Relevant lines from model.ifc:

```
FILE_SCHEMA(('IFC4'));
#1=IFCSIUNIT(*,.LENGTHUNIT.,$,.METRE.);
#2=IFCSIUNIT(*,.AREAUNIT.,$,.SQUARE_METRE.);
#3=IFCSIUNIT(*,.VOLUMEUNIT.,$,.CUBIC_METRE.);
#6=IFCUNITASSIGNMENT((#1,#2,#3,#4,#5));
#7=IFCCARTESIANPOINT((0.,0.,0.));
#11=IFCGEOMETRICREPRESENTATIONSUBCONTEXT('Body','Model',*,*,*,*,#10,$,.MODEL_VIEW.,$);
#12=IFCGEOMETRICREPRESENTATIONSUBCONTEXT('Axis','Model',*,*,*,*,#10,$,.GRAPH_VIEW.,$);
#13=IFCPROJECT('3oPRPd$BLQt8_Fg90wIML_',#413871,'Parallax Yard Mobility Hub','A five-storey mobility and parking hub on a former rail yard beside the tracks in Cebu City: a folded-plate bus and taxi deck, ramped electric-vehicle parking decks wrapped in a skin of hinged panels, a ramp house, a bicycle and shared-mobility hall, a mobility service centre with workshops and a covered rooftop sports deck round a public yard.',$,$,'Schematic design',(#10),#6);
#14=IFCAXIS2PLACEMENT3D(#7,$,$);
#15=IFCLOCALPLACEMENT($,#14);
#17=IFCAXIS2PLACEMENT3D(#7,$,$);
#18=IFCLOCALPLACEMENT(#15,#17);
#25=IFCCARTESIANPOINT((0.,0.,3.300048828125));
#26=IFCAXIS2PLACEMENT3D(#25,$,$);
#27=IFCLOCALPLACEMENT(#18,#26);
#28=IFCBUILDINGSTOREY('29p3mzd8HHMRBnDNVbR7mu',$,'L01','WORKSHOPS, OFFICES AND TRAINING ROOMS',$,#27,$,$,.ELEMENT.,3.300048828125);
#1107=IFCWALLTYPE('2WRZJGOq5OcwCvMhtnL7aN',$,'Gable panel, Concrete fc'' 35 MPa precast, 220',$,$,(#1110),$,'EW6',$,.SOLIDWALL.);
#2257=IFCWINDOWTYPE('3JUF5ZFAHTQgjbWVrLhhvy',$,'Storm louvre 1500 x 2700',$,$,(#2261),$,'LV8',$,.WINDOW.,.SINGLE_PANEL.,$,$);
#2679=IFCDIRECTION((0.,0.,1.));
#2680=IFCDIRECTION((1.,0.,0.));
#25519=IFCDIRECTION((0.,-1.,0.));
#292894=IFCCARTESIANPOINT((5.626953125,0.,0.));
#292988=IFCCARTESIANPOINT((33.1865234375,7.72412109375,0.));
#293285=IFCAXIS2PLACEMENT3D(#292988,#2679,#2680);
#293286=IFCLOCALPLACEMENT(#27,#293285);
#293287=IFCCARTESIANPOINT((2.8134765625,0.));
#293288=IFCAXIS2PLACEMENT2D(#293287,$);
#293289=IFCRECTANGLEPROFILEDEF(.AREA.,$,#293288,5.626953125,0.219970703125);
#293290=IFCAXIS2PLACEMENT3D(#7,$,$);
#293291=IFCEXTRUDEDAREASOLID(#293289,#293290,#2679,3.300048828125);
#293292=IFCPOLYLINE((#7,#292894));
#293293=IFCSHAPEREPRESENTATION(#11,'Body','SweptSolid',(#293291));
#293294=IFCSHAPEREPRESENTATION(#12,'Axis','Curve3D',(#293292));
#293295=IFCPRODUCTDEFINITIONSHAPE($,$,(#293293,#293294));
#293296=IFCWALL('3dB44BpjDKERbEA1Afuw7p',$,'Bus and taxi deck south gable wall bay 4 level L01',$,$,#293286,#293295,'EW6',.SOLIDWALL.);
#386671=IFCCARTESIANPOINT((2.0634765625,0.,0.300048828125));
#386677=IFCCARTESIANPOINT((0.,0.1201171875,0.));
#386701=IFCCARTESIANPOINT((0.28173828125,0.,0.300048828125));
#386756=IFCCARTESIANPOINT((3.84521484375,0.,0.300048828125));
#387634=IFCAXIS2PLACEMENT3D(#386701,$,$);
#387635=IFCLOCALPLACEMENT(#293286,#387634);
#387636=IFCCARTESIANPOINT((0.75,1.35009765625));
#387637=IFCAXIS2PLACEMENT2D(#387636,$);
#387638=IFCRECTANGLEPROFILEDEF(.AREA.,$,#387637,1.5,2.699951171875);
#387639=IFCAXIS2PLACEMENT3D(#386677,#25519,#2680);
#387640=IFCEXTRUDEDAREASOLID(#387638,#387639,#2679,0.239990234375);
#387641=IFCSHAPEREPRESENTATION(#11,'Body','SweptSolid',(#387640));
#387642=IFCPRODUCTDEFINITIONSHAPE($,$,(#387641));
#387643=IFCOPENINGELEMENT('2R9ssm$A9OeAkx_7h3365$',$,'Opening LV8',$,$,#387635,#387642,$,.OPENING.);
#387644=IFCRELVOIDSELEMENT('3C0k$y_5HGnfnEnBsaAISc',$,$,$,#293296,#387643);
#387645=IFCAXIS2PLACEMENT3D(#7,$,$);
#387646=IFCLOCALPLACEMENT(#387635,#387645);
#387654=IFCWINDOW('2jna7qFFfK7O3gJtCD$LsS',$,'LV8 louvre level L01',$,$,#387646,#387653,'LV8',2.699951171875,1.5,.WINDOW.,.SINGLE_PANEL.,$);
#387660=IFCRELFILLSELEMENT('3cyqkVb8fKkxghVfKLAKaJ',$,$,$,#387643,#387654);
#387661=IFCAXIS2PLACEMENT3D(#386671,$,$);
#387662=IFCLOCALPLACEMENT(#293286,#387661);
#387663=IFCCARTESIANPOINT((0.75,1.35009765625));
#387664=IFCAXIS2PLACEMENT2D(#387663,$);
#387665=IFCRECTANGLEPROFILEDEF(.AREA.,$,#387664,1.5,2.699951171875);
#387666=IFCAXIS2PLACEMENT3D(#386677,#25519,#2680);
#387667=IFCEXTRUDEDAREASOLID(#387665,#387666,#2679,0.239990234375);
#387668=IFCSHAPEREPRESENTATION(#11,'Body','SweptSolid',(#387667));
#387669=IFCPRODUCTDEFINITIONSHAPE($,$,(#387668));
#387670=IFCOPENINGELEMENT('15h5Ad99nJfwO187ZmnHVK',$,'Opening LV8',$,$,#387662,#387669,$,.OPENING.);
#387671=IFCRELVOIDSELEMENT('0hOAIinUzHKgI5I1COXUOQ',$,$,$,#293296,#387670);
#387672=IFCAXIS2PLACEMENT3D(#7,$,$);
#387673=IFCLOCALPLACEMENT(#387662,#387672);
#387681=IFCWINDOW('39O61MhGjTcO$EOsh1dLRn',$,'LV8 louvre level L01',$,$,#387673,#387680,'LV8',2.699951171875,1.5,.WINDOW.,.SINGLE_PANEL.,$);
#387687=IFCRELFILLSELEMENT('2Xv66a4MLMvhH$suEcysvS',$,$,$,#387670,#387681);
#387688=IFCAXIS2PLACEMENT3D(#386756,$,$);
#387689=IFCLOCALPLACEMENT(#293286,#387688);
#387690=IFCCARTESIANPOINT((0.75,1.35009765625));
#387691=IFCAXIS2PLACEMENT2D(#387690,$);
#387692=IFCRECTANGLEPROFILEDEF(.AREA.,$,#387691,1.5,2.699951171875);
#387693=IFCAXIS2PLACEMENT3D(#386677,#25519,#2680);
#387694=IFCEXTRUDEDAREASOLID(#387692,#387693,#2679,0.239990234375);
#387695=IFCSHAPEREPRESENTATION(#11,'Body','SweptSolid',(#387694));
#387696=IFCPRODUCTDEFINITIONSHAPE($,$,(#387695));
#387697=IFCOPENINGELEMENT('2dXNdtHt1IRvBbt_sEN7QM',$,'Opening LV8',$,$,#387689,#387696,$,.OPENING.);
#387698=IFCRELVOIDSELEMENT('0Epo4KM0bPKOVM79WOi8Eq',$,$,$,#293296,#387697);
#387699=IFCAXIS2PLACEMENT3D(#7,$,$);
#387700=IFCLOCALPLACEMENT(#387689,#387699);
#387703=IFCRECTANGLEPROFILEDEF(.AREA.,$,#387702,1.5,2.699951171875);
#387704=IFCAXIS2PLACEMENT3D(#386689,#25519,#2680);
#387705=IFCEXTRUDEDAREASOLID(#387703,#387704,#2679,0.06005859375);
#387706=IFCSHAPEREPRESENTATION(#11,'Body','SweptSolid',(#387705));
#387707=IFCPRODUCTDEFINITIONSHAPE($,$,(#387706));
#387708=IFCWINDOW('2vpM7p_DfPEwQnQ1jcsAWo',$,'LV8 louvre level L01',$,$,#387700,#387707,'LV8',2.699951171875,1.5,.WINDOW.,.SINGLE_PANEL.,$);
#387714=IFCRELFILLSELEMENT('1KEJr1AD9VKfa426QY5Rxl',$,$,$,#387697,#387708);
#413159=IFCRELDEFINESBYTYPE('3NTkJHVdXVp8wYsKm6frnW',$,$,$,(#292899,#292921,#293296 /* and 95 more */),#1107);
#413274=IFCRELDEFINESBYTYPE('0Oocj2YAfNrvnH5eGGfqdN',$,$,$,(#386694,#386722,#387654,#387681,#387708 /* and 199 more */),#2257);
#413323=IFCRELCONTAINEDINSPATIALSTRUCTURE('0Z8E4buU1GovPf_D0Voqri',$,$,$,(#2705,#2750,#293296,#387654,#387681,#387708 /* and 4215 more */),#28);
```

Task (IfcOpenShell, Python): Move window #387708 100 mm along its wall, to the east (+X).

```python
import ifcopenshell
import ifcopenshell.api.geometry
import ifcopenshell.util.placement

model = ifcopenshell.open("model.ifc")

window = model.by_id(387708)
opening = window.FillsVoids[0].RelatingOpeningElement
wall = opening.VoidsElements[0].RelatingBuildingElement

wall_matrix = ifcopenshell.util.placement.get_local_placement(wall.ObjectPlacement)
shift = wall_matrix[:3, 0] * 0.1
before = ifcopenshell.util.placement.get_local_placement(window.ObjectPlacement)[:3, 3].copy()

# The window is placed relative to its opening, so it follows when the opening moves.
matrix = ifcopenshell.util.placement.get_local_placement(opening.ObjectPlacement)
matrix[:3, 3] += shift
ifcopenshell.api.geometry.edit_object_placement(
    model, product=opening, matrix=matrix, is_si=False, should_transform_children=True
)

after = ifcopenshell.util.placement.get_local_placement(window.ObjectPlacement)[:3, 3]
print("window moved by", (after - before).round(3) + 0.0)

model.write("model_updated.ifc")
```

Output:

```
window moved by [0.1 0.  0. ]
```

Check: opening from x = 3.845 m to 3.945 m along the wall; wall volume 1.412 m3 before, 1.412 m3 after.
